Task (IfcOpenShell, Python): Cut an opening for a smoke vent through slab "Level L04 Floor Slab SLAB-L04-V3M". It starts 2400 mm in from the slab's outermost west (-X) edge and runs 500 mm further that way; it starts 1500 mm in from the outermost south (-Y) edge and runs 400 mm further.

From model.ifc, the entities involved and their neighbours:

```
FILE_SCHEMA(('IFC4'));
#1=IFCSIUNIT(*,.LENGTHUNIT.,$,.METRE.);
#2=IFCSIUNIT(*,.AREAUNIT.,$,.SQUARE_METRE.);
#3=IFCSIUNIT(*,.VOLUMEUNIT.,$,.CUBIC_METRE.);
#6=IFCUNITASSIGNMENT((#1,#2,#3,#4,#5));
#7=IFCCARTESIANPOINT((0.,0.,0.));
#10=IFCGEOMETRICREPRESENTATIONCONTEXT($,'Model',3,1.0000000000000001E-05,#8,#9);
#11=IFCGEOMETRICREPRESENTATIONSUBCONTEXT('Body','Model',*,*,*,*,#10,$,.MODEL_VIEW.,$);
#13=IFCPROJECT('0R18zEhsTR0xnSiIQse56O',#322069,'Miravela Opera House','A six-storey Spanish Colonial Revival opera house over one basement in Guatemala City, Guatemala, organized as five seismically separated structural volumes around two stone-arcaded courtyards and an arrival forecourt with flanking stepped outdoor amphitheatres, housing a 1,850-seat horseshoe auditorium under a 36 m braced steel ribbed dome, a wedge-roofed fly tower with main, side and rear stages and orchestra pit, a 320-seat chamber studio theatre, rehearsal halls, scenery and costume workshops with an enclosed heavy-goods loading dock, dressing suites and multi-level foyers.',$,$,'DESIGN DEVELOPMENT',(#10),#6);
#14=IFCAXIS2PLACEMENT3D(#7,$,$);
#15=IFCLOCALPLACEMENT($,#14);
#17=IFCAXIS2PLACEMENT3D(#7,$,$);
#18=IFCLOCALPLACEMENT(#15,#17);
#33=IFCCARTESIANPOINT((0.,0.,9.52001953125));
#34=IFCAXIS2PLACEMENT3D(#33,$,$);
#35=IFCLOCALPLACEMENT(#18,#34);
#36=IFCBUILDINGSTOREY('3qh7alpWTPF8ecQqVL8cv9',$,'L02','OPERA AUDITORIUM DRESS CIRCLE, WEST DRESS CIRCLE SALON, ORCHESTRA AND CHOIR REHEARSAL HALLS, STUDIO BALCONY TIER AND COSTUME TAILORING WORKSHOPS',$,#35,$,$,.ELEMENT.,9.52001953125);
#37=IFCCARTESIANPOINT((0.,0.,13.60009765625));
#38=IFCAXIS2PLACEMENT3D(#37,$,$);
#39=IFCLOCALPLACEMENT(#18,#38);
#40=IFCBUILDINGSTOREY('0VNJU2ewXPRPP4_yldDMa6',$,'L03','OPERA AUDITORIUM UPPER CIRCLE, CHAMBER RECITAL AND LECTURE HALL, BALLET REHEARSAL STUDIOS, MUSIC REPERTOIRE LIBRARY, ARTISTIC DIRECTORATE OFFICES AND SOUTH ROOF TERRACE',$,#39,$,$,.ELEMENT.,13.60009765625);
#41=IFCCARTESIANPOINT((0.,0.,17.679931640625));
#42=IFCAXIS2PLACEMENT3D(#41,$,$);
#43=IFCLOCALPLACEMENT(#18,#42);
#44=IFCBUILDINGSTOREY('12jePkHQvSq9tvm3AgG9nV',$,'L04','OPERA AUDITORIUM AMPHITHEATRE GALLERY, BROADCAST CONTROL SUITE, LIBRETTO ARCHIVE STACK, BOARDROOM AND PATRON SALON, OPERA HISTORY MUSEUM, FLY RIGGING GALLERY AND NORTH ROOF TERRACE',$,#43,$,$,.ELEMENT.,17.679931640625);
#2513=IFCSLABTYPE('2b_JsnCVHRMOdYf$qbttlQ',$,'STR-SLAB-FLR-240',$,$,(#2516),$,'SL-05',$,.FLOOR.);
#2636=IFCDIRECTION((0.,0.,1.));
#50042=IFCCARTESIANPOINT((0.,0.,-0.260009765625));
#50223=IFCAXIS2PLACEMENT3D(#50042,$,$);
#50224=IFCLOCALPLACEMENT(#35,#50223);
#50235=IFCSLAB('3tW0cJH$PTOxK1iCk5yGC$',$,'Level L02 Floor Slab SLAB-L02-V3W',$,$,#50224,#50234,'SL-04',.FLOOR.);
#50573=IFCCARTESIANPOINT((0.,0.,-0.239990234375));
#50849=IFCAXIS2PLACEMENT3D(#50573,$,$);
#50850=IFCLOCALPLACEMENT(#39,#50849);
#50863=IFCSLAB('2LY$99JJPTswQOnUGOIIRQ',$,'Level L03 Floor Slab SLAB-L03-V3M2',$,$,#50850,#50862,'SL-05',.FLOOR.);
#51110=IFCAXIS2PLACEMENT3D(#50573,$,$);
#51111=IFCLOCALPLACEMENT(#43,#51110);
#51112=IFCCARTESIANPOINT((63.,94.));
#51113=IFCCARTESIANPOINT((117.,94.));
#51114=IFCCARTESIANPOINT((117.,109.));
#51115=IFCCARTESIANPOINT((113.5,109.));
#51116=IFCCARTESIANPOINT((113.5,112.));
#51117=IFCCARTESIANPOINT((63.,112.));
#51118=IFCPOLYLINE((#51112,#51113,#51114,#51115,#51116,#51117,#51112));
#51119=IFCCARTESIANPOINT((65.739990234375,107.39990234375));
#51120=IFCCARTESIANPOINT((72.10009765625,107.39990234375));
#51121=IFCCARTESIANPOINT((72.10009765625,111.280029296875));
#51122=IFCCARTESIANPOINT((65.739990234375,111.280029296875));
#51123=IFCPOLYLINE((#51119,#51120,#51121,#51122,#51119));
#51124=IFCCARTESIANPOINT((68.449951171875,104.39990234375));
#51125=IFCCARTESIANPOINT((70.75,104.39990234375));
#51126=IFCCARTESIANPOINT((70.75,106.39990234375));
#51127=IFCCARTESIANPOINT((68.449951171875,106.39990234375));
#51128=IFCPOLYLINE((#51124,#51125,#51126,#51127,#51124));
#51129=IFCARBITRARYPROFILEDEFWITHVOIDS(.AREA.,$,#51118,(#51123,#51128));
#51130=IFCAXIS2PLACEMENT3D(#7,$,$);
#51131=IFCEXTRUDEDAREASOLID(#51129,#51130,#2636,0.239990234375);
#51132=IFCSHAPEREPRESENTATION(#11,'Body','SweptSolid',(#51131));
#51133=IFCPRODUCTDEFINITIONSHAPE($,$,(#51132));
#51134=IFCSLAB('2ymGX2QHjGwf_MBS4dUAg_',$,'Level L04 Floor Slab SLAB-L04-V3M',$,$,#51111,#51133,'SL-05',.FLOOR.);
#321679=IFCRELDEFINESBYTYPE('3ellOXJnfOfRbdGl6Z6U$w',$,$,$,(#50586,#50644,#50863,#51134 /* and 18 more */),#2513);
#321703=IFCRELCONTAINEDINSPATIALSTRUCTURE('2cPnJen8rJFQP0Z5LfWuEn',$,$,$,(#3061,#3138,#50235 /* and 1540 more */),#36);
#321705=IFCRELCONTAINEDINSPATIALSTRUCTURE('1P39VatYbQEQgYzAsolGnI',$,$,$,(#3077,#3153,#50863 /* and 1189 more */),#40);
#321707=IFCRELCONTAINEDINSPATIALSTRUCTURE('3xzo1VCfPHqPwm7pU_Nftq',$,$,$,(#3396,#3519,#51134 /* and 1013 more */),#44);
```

```python
import numpy as np
import ifcopenshell
import ifcopenshell.api.feature
import ifcopenshell.api.geometry
import ifcopenshell.api.root
import ifcopenshell.geom
import ifcopenshell.util.placement
import ifcopenshell.util.representation
import ifcopenshell.util.shape
import ifcopenshell.util.unit

model = ifcopenshell.open("model.ifc")
unit_scale = ifcopenshell.util.unit.calculate_unit_scale(model)
settings = ifcopenshell.geom.settings()


def volume(element):
    """Net volume in cubic metres, openings subtracted."""
    shape = ifcopenshell.geom.create_shape(settings, element)
    return ifcopenshell.util.shape.get_volume(shape.geometry)


slab = model.by_guid("2ymGX2QHjGwf_MBS4dUAg_")
before = volume(slab)

# Extent in the slab's own axes, in metres. The edges named are its -X and -Y sides.
slab_shape = ifcopenshell.geom.create_shape(settings, slab)
vertices = ifcopenshell.util.shape.get_vertices(slab_shape.geometry)
x_min, y_min, bottom = vertices.min(axis=0)
top = vertices[:, 2].max()

opening = ifcopenshell.api.root.create_entity(model, ifc_class="IfcOpeningElement", name="Smoke vent opening", predefined_type="OPENING")
context = ifcopenshell.util.representation.get_context(model, "Model", "Body", "MODEL_VIEW")
width, depth = 0.5, 0.4
outline = [(0.0, 0.0), (width, 0.0), (width, depth), (0.0, depth), (0.0, 0.0)]
# Overshoot both faces by 50 mm so the cut is clean.
shape = ifcopenshell.api.geometry.add_slab_representation(
    model, context=context, depth=top - bottom + 0.1, polyline=outline
)
ifcopenshell.api.geometry.assign_representation(model, product=opening, representation=shape)

matrix = ifcopenshell.util.placement.get_local_placement(slab.ObjectPlacement)
matrix[:, 3] = matrix @ np.append(np.array([x_min + 2.4, y_min + 1.5, bottom - 0.05]) / unit_scale, 1.0)
ifcopenshell.api.geometry.edit_object_placement(model, product=opening, matrix=matrix, is_si=False)
ifcopenshell.api.feature.add_feature(model, feature=opening, element=slab)

after = volume(slab)

print(f"slab volume {before:.3f} -> {after:.3f} m3")

model.write("model_edited.ifc")
```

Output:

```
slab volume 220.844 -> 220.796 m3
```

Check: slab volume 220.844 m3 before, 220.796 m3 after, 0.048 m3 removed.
